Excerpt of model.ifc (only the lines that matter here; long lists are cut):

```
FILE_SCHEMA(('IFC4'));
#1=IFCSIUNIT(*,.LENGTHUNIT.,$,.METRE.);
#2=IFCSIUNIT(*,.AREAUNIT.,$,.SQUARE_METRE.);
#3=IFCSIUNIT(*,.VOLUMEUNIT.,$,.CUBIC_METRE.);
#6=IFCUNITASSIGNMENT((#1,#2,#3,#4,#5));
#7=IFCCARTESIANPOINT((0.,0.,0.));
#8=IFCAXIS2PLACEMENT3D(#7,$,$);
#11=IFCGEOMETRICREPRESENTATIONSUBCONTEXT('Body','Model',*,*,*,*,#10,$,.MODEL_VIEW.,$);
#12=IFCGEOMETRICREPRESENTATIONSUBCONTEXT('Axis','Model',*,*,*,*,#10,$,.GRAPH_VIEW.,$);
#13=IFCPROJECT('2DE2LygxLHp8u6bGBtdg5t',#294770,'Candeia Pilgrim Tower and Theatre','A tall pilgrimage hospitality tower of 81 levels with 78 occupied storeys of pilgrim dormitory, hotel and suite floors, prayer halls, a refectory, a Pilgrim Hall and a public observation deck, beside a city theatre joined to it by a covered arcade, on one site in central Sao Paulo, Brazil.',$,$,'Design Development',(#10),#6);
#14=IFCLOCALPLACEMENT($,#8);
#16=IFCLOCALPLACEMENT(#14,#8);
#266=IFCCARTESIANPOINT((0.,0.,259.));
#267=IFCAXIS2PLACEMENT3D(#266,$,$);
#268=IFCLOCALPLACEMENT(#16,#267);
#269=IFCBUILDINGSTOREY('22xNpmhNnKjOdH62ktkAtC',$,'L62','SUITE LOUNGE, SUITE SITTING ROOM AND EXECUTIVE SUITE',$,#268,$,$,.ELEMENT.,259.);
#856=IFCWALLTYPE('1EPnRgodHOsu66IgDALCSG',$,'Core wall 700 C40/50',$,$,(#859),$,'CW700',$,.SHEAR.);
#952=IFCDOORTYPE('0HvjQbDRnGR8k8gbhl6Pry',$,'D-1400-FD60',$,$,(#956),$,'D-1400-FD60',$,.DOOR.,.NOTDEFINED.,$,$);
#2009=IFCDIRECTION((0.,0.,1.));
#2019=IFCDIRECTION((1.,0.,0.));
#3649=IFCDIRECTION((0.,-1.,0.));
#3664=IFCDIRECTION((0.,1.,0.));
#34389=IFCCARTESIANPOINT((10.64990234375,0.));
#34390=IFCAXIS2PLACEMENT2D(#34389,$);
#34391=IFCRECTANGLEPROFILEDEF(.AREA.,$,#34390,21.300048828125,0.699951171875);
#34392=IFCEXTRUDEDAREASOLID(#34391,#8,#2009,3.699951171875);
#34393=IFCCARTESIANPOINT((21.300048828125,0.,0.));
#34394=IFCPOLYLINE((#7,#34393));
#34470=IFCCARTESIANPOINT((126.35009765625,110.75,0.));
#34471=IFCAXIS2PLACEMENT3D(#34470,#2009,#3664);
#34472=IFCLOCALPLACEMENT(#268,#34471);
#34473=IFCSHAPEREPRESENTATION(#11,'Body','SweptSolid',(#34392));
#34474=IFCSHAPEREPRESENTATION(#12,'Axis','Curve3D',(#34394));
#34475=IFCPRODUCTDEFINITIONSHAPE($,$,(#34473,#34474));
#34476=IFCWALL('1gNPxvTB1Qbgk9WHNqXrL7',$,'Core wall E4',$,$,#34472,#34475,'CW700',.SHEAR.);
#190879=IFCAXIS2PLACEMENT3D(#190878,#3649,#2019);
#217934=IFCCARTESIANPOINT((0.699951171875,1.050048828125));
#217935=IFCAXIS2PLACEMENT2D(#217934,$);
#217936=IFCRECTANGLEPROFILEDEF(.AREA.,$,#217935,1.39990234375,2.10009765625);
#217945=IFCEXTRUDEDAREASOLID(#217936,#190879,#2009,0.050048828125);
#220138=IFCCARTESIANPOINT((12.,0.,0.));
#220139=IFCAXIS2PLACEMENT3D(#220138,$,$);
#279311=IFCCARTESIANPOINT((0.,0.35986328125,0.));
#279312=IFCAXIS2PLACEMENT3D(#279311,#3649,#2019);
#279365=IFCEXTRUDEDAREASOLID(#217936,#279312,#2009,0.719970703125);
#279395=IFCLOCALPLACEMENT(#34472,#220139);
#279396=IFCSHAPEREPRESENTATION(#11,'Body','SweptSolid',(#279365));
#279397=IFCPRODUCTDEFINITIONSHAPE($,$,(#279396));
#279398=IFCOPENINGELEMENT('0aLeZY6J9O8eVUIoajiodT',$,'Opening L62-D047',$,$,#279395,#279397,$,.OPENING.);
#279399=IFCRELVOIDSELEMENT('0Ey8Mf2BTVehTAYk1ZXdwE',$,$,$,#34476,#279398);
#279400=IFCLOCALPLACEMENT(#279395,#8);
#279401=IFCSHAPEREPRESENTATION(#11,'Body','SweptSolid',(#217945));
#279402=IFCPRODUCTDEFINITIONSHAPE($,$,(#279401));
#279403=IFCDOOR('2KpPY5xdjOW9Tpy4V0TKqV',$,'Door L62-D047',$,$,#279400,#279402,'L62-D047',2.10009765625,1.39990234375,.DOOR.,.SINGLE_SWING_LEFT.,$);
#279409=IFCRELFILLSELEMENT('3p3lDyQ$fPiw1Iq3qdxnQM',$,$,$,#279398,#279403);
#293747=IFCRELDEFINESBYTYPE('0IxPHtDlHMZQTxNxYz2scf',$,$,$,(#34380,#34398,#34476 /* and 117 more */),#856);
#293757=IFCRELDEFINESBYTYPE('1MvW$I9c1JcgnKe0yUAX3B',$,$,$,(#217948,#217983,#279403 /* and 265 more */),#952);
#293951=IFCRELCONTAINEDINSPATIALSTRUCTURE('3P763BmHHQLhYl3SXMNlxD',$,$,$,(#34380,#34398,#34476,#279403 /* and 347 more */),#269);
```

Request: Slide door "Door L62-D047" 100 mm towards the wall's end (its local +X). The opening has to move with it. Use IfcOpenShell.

```python
import ifcopenshell
import ifcopenshell.api.geometry
import ifcopenshell.util.placement
import ifcopenshell.util.unit

model = ifcopenshell.open("model.ifc")
unit_scale = ifcopenshell.util.unit.calculate_unit_scale(model)

door = model.by_guid("2KpPY5xdjOW9Tpy4V0TKqV")
opening = door.FillsVoids[0].RelatingOpeningElement
wall = opening.VoidsElements[0].RelatingBuildingElement

wall_matrix = ifcopenshell.util.placement.get_local_placement(wall.ObjectPlacement)
shift = wall_matrix[:3, 0] * 0.1 / unit_scale
before = ifcopenshell.util.placement.get_local_placement(door.ObjectPlacement)[:3, 3].copy()

# The door is placed relative to its opening, so it follows when the opening moves.
matrix = ifcopenshell.util.placement.get_local_placement(opening.ObjectPlacement)
matrix[:3, 3] += shift
ifcopenshell.api.geometry.edit_object_placement(
    model, product=opening, matrix=matrix, is_si=False, should_transform_children=True
)

after = ifcopenshell.util.placement.get_local_placement(door.ObjectPlacement)[:3, 3]
print("door moved by", (after - before).round(3) + 0.0)

model.write("model_edited.ifc")
```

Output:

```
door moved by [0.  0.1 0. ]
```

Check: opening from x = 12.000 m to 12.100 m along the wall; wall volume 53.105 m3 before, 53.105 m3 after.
